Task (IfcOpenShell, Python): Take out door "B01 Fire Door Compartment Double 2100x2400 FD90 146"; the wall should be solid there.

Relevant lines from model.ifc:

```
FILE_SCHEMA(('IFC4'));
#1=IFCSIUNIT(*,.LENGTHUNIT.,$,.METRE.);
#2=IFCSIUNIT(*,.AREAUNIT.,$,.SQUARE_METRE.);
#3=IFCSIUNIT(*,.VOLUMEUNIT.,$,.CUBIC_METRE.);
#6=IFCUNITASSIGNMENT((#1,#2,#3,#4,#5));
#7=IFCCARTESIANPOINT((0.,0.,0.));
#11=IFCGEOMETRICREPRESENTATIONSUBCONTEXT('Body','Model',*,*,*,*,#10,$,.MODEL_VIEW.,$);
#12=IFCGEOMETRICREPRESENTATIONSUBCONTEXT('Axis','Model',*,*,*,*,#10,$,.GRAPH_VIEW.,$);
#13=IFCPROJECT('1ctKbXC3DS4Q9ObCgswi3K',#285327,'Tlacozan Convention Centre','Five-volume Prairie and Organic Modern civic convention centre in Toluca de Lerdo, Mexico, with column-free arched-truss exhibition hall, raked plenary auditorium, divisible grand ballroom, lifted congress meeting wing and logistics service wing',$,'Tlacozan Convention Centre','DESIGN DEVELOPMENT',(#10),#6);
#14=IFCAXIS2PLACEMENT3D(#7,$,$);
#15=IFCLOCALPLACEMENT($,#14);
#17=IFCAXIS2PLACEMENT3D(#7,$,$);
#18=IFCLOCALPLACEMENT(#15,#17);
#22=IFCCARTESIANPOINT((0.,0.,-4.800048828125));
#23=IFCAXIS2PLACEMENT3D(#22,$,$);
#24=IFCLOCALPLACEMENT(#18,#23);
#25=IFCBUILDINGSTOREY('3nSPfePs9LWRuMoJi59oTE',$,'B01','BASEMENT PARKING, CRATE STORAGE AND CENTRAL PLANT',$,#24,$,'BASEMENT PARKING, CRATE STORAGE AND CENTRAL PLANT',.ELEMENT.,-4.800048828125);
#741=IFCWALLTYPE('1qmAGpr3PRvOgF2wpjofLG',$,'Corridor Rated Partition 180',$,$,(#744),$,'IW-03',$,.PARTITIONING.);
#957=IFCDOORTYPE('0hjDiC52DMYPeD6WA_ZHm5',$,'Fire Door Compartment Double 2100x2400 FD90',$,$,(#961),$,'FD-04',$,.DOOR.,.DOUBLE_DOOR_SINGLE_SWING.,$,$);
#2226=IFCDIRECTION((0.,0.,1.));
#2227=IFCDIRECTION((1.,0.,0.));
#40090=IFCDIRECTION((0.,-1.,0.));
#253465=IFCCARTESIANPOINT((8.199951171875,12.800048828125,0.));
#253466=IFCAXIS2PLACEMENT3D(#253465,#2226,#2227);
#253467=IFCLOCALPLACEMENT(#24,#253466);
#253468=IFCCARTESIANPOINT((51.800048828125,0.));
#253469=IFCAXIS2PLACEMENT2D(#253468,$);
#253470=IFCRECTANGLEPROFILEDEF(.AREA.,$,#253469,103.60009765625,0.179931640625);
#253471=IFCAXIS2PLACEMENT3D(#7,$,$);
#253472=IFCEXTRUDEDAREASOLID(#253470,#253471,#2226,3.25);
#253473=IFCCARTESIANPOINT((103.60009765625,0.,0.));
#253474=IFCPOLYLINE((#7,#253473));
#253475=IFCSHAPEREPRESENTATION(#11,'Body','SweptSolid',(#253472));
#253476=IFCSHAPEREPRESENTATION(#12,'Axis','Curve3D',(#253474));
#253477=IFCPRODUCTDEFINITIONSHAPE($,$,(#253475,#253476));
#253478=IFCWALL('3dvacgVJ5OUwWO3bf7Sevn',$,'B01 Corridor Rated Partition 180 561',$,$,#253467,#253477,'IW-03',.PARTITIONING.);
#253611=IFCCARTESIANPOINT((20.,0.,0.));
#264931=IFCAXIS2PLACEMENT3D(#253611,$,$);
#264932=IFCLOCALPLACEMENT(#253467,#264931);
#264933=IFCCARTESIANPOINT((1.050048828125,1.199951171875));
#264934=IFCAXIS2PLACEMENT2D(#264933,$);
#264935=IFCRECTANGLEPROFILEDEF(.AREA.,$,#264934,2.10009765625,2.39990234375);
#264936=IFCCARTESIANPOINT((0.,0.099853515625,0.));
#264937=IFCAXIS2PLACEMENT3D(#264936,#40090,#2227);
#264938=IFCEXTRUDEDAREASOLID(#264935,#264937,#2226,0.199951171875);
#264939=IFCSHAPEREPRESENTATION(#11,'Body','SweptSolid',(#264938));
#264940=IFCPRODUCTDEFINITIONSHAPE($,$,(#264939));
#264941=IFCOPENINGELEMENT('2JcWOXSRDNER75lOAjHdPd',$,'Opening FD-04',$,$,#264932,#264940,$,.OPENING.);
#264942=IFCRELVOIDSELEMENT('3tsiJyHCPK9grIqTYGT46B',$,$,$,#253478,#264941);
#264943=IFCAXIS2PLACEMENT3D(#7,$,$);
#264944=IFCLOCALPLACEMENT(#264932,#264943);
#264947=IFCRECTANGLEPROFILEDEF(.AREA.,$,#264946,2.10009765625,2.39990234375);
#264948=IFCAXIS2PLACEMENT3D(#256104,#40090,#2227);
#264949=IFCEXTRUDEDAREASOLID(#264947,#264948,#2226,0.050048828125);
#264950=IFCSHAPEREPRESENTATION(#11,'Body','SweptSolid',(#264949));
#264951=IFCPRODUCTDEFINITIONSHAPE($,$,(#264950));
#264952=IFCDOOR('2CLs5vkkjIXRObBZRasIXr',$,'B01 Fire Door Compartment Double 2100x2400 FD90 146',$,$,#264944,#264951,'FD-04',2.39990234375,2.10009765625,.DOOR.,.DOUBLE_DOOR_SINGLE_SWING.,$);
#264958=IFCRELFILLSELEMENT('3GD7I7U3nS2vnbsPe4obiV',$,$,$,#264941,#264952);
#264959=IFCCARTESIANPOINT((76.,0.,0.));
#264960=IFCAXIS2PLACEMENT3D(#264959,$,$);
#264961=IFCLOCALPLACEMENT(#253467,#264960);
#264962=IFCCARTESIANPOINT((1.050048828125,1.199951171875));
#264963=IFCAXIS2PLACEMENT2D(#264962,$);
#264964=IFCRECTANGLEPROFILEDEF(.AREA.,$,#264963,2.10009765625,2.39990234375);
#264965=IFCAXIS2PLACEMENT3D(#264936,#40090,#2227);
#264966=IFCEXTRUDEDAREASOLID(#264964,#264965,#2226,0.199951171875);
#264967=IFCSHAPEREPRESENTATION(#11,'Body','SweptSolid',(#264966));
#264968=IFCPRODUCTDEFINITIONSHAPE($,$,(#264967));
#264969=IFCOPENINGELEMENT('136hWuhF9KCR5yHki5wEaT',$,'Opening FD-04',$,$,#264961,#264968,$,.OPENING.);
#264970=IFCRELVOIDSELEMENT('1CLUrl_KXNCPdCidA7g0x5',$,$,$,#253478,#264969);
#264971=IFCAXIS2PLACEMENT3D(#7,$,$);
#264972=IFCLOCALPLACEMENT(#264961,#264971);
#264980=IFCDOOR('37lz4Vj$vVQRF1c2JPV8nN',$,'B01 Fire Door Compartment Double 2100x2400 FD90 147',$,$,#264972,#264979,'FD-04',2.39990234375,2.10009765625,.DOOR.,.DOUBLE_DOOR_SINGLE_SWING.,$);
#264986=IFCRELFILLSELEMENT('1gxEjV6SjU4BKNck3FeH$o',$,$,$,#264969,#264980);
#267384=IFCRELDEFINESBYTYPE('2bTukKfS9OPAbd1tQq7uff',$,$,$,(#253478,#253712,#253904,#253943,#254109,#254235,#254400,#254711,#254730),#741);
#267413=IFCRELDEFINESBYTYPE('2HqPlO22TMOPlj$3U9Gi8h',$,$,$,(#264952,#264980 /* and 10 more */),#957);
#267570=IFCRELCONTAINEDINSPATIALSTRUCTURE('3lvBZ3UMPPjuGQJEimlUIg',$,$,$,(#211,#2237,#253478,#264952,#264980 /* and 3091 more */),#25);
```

```python
import ifcopenshell
import ifcopenshell.api.feature
import ifcopenshell.api.root
import ifcopenshell.geom
import ifcopenshell.util.shape

model = ifcopenshell.open("model.ifc")
settings = ifcopenshell.geom.settings()


def volume(element):
    """Net volume in cubic metres, openings subtracted."""
    shape = ifcopenshell.geom.create_shape(settings, element)
    return ifcopenshell.util.shape.get_volume(shape.geometry)


door = model.by_id(264952)
opening = door.FillsVoids[0].RelatingOpeningElement
wall = opening.VoidsElements[0].RelatingBuildingElement
before = volume(wall)

ifcopenshell.api.root.remove_product(model, product=door)
ifcopenshell.api.feature.remove_feature(model, feature=opening)

after = volume(wall)

print(f"wall volume {before:.3f} -> {after:.3f} m3")

model.write("model-out.ifc")
```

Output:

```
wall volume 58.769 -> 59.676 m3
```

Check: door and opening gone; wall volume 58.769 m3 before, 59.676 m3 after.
